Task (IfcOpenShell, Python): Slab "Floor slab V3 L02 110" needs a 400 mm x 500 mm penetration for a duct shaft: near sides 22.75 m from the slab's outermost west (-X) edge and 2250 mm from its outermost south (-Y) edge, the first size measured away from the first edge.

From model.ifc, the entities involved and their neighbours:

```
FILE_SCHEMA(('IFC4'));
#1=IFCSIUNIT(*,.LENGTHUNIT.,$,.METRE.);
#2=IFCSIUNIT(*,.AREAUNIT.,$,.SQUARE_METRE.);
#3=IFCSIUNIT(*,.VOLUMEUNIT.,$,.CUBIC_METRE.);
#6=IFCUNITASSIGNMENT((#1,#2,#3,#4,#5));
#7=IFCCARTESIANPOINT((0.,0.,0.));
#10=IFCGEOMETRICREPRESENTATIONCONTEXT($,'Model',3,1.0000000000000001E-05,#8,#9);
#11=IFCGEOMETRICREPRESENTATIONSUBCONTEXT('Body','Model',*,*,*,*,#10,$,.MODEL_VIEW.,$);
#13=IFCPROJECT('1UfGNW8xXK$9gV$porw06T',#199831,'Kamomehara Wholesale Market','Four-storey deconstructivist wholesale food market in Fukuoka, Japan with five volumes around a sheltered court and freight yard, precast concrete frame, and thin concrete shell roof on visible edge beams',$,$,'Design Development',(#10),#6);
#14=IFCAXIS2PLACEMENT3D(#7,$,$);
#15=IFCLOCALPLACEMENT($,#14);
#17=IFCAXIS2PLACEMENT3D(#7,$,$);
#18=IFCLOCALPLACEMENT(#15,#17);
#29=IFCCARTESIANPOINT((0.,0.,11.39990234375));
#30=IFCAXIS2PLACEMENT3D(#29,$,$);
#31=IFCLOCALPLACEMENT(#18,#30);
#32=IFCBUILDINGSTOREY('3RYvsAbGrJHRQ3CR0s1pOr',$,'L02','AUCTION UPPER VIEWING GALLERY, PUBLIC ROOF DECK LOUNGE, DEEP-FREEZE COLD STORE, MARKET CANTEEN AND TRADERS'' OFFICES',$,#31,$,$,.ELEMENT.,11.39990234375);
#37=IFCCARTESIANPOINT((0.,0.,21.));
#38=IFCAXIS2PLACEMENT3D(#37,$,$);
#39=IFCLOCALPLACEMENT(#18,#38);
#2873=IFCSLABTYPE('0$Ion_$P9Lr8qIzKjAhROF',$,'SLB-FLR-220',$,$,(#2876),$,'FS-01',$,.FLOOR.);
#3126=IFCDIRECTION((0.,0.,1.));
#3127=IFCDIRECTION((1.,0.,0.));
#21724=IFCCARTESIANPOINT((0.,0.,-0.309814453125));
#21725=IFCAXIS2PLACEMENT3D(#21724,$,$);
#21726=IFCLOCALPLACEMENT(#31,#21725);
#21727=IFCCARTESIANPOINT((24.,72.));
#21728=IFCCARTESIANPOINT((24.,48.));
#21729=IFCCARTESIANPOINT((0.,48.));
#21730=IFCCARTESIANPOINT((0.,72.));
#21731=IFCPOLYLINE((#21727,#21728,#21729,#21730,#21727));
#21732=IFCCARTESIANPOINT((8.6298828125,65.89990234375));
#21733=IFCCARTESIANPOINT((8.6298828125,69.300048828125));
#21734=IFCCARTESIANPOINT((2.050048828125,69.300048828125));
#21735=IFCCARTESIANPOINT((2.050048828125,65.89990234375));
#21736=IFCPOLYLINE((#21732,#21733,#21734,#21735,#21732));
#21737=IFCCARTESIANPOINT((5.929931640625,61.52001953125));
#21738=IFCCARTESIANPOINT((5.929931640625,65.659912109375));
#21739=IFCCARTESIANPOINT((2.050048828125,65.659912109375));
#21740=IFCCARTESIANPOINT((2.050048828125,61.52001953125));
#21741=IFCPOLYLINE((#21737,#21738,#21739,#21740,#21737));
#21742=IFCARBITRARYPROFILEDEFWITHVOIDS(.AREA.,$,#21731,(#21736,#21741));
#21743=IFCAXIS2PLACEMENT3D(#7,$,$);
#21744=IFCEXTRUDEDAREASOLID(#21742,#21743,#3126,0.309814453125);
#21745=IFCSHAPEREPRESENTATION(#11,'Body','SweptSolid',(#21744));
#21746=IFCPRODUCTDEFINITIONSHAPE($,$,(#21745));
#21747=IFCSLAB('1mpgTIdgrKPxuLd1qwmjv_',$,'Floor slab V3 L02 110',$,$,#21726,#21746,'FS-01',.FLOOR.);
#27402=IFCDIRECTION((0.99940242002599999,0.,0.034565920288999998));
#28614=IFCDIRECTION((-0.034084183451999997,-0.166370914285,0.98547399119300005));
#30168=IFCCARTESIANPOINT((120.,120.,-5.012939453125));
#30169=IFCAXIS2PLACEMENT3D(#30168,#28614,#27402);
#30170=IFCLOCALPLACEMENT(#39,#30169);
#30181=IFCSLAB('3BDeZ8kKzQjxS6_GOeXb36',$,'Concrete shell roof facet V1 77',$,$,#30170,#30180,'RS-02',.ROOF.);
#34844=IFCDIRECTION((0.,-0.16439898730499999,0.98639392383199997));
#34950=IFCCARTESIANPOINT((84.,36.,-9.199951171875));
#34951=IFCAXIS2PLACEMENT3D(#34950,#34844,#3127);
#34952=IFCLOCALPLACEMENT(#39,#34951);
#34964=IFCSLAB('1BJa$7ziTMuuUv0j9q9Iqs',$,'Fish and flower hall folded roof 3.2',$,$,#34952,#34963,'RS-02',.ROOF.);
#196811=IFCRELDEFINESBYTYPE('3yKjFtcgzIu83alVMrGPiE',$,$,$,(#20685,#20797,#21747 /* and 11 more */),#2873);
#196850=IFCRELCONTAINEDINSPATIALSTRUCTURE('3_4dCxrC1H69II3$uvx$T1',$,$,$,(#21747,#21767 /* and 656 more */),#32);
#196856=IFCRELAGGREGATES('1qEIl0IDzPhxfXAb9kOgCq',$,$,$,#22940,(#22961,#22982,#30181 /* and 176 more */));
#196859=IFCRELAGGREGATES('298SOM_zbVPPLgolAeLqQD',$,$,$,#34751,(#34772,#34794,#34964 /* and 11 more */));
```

```python
import numpy as np
import ifcopenshell
import ifcopenshell.api.feature
import ifcopenshell.api.geometry
import ifcopenshell.api.root
import ifcopenshell.geom
import ifcopenshell.util.placement
import ifcopenshell.util.representation
import ifcopenshell.util.shape
import ifcopenshell.util.unit

model = ifcopenshell.open("model.ifc")
unit_scale = ifcopenshell.util.unit.calculate_unit_scale(model)
settings = ifcopenshell.geom.settings()


def volume(element):
    """Net volume in cubic metres, openings subtracted."""
    shape = ifcopenshell.geom.create_shape(settings, element)
    return ifcopenshell.util.shape.get_volume(shape.geometry)


slab = model.by_guid("1mpgTIdgrKPxuLd1qwmjv_")
before = volume(slab)

# Extent in the slab's own axes, in metres. The edges named are its -X and -Y sides.
slab_shape = ifcopenshell.geom.create_shape(settings, slab)
vertices = ifcopenshell.util.shape.get_vertices(slab_shape.geometry)
x_min, y_min, bottom = vertices.min(axis=0)
top = vertices[:, 2].max()

opening = ifcopenshell.api.root.create_entity(model, ifc_class="IfcOpeningElement", name="Duct shaft opening", predefined_type="OPENING")
context = ifcopenshell.util.representation.get_context(model, "Model", "Body", "MODEL_VIEW")
width, depth = 0.4, 0.5
outline = [(0.0, 0.0), (width, 0.0), (width, depth), (0.0, depth), (0.0, 0.0)]
# Overshoot both faces by 50 mm so the cut is clean.
shape = ifcopenshell.api.geometry.add_slab_representation(
    model, context=context, depth=top - bottom + 0.1, polyline=outline
)
ifcopenshell.api.geometry.assign_representation(model, product=opening, representation=shape)

matrix = ifcopenshell.util.placement.get_local_placement(slab.ObjectPlacement)
matrix[:, 3] = matrix @ np.append(np.array([x_min + 22.75, y_min + 2.25, bottom - 0.05]) / unit_scale, 1.0)
ifcopenshell.api.geometry.edit_object_placement(model, product=opening, matrix=matrix, is_si=False)
ifcopenshell.api.feature.add_feature(model, feature=opening, element=slab)

after = volume(slab)

print(f"slab volume {before:.3f} -> {after:.3f} m3")

model.write("model_rev.ifc")
```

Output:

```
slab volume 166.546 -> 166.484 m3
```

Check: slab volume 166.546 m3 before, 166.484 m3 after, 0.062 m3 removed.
